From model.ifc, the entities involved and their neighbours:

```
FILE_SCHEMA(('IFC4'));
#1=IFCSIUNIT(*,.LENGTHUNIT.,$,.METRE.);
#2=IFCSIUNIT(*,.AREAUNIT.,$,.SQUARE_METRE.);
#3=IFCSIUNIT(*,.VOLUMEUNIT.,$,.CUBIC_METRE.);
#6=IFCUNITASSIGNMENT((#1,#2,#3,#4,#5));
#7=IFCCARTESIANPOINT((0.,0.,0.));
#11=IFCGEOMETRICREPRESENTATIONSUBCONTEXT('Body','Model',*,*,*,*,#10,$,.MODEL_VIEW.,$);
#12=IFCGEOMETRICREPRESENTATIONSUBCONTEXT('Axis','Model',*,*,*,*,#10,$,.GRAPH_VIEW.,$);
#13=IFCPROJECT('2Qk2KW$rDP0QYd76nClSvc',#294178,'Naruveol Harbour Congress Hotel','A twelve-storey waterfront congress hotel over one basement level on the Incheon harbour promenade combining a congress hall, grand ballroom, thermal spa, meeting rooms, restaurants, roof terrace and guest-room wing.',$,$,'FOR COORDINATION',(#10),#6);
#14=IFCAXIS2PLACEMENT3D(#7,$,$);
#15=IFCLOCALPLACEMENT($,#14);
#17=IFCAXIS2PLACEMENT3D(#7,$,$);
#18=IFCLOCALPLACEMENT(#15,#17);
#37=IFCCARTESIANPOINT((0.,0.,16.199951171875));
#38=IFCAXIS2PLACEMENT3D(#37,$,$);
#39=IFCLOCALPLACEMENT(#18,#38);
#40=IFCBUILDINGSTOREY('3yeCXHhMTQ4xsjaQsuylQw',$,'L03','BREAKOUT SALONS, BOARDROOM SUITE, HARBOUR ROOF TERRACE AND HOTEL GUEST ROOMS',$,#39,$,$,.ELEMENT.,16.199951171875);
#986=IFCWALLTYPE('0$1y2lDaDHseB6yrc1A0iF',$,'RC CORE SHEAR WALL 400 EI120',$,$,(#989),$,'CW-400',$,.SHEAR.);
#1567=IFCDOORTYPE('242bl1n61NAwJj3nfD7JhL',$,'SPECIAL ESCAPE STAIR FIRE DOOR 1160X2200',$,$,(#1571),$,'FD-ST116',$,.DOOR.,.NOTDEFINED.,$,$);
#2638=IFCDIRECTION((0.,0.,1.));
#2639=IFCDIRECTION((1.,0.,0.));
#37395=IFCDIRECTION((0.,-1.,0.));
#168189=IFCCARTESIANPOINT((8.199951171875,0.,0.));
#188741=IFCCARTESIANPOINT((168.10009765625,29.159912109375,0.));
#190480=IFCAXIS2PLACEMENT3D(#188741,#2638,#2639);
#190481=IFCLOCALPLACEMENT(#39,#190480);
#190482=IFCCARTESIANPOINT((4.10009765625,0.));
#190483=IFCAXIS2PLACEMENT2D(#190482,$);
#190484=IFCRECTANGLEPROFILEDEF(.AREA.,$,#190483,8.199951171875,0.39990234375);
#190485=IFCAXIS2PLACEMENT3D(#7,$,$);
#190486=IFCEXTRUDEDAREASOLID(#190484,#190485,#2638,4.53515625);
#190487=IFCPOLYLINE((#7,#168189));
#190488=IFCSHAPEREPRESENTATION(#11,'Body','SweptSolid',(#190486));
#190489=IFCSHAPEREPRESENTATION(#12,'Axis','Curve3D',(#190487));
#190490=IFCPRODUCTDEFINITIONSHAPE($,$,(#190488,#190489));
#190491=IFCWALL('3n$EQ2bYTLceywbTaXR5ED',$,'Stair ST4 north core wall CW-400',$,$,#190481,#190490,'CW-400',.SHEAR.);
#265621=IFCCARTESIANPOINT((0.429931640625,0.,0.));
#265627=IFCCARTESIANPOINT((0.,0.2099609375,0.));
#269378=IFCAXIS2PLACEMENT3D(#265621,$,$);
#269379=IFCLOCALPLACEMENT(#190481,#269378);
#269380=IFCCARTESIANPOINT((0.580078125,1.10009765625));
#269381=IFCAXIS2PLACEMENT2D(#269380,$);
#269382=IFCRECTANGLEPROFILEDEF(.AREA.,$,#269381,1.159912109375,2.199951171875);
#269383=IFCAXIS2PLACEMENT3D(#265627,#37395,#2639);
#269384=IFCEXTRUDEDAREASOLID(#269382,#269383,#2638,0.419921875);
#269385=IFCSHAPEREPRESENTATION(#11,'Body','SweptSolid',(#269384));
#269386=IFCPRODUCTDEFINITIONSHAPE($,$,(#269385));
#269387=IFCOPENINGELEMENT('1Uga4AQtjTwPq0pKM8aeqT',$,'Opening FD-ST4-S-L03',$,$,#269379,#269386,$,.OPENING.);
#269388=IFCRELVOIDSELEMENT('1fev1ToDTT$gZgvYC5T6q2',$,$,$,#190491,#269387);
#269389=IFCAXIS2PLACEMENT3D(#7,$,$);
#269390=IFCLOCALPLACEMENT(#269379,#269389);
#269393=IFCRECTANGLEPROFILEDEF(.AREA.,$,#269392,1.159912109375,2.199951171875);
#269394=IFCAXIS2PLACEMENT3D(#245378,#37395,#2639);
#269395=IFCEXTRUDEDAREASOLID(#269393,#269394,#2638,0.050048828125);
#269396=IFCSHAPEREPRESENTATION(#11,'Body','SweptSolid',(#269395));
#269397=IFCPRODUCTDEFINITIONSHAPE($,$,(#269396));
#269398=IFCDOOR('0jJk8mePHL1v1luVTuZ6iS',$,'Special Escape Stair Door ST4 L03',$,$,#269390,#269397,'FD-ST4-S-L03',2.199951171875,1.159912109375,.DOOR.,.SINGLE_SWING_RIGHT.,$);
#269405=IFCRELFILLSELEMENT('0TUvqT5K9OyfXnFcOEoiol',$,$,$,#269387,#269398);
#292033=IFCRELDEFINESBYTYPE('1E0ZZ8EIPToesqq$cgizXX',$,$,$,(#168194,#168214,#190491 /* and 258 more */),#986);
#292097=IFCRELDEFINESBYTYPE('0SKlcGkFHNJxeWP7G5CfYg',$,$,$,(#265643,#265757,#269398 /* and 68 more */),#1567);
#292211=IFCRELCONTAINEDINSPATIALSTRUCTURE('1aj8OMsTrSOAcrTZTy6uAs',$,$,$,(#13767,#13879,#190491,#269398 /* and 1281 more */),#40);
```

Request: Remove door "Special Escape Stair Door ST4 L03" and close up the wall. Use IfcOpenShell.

```python
import ifcopenshell
import ifcopenshell.api.feature
import ifcopenshell.api.root
import ifcopenshell.geom
import ifcopenshell.util.shape

model = ifcopenshell.open("model.ifc")
settings = ifcopenshell.geom.settings()


def volume(element):
    """Net volume in cubic metres, openings subtracted."""
    shape = ifcopenshell.geom.create_shape(settings, element)
    return ifcopenshell.util.shape.get_volume(shape.geometry)


door = model.by_id(269398)
opening = door.FillsVoids[0].RelatingOpeningElement
wall = opening.VoidsElements[0].RelatingBuildingElement
before = volume(wall)

ifcopenshell.api.root.remove_product(model, product=door)
ifcopenshell.api.feature.remove_feature(model, feature=opening)

after = volume(wall)

print(f"wall volume {before:.3f} -> {after:.3f} m3")

model.write("model_v2.ifc")
```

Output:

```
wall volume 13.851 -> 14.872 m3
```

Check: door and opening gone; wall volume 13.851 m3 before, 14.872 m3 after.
